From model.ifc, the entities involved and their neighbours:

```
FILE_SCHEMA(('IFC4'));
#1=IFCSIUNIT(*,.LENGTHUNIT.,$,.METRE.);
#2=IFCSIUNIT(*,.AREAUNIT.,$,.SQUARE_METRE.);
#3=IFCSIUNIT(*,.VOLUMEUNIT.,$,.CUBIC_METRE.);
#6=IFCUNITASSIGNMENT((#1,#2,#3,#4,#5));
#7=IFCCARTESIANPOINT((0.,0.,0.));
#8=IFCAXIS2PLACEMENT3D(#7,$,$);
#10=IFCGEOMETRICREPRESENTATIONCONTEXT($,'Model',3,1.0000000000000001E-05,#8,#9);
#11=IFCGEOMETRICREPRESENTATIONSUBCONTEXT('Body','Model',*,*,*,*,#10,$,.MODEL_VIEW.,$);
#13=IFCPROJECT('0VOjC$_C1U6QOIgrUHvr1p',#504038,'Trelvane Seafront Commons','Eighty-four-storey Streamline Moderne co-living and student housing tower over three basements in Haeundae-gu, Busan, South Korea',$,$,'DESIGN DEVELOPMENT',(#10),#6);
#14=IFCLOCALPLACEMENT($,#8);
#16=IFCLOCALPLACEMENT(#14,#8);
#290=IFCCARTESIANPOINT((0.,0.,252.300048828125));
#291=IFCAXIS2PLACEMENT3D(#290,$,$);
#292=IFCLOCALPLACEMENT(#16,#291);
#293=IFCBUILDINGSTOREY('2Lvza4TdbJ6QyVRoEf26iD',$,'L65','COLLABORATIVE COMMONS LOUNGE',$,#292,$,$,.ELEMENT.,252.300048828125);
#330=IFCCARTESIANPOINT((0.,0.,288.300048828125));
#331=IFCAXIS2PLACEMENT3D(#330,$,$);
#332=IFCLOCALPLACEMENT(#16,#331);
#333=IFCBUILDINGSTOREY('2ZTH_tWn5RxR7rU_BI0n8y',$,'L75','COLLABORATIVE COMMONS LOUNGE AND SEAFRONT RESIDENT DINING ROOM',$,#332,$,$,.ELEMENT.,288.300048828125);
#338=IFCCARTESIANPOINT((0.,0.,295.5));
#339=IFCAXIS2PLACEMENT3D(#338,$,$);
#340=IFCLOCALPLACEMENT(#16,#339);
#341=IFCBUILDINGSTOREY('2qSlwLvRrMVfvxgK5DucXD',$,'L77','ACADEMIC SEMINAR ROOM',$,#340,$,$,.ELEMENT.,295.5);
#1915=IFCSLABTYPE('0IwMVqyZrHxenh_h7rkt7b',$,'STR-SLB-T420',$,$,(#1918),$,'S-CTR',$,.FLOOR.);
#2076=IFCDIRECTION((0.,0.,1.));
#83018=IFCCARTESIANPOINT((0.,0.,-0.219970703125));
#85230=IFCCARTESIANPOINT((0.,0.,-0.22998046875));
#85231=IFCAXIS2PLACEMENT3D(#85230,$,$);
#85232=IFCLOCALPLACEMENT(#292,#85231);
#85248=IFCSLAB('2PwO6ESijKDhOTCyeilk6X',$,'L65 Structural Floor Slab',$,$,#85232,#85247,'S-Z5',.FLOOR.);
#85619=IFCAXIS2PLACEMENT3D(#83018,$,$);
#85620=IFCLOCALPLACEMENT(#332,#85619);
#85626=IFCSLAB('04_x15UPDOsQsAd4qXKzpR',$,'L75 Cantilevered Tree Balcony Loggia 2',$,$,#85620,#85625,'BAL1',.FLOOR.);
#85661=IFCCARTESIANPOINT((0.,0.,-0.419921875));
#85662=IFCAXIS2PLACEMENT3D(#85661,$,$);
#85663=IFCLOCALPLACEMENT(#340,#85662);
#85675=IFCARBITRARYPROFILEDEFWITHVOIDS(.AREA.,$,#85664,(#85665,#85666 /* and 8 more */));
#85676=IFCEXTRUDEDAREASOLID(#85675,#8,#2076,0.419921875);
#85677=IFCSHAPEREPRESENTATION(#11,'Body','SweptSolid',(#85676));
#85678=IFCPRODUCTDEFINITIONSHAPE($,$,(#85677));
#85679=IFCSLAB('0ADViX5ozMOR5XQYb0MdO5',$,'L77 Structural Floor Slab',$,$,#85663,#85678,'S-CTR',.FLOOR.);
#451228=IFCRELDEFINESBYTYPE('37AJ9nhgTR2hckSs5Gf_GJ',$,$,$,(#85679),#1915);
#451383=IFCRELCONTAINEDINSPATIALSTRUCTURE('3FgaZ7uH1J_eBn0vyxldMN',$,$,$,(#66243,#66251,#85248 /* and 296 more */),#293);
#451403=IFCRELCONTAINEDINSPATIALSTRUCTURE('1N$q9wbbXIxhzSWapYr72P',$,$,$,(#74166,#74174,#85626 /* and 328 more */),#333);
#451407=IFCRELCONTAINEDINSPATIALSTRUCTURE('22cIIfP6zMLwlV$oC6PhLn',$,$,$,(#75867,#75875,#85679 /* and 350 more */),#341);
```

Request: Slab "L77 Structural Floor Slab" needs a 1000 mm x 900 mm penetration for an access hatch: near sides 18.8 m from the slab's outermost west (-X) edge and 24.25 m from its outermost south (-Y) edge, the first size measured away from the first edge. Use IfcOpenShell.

```python
import numpy as np
import ifcopenshell
import ifcopenshell.api.feature
import ifcopenshell.api.geometry
import ifcopenshell.api.root
import ifcopenshell.geom
import ifcopenshell.util.placement
import ifcopenshell.util.representation
import ifcopenshell.util.shape
import ifcopenshell.util.unit

model = ifcopenshell.open("model.ifc")
unit_scale = ifcopenshell.util.unit.calculate_unit_scale(model)
settings = ifcopenshell.geom.settings()


def volume(element):
    """Net volume in cubic metres, openings subtracted."""
    shape = ifcopenshell.geom.create_shape(settings, element)
    return ifcopenshell.util.shape.get_volume(shape.geometry)


slab = model.by_id(85679)
before = volume(slab)

# Extent in the slab's own axes, in metres. The edges named are its -X and -Y sides.
slab_shape = ifcopenshell.geom.create_shape(settings, slab)
vertices = ifcopenshell.util.shape.get_vertices(slab_shape.geometry)
x_min, y_min, bottom = vertices.min(axis=0)
top = vertices[:, 2].max()

opening = ifcopenshell.api.root.create_entity(model, ifc_class="IfcOpeningElement", name="Access hatch opening", predefined_type="OPENING")
context = ifcopenshell.util.representation.get_context(model, "Model", "Body", "MODEL_VIEW")
width, depth = 1, 0.9
outline = [(0.0, 0.0), (width, 0.0), (width, depth), (0.0, depth), (0.0, 0.0)]
# Overshoot both faces by 50 mm so the cut is clean.
shape = ifcopenshell.api.geometry.add_slab_representation(
    model, context=context, depth=top - bottom + 0.1, polyline=outline
)
ifcopenshell.api.geometry.assign_representation(model, product=opening, representation=shape)

matrix = ifcopenshell.util.placement.get_local_placement(slab.ObjectPlacement)
matrix[:, 3] = matrix @ np.append(np.array([x_min + 18.8, y_min + 24.25, bottom - 0.05]) / unit_scale, 1.0)
ifcopenshell.api.geometry.edit_object_placement(model, product=opening, matrix=matrix, is_si=False)
ifcopenshell.api.feature.add_feature(model, feature=opening, element=slab)

after = volume(slab)

print(f"slab volume {before:.3f} -> {after:.3f} m3")

model.write("model_edited.ifc")
```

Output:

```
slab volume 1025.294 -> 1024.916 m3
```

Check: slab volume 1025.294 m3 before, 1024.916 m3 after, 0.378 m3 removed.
